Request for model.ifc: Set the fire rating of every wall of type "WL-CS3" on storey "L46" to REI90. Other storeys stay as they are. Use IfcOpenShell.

First a look at what the model holds.

```python
import ifcopenshell
import ifcopenshell.util.element

model = ifcopenshell.open("model.ifc")
print(model.schema)
storey = next(s for s in model.by_type("IfcBuildingStorey") if s.Name == "L46")
walls = [e for e in ifcopenshell.util.element.get_decomposition(storey) if e.is_a("IfcWall")]
seen = {}
for e in walls:
    element_type = ifcopenshell.util.element.get_type(e)
    key = (element_type.Name if element_type != e and element_type else None, ifcopenshell.util.element.get_pset(e, "Pset_WallCommon", "FireRating"))
    seen[key] = seen.get(key, 0) + 1
for (name, value), count in sorted(seen.items(), key=str):
    print(count, "x", name, "|", value)
```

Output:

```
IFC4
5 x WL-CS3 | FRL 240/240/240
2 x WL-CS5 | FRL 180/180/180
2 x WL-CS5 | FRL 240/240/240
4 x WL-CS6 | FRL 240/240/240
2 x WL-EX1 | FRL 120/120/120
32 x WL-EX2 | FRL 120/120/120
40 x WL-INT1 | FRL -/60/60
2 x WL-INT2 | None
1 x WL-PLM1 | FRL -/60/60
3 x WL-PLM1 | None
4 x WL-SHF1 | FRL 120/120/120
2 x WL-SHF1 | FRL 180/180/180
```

```python
import ifcopenshell
import ifcopenshell.api.pset
import ifcopenshell.util.element

model = ifcopenshell.open("model.ifc")

storey = next(s for s in model.by_type("IfcBuildingStorey") if s.Name == "L46")
walls = [e for e in ifcopenshell.util.element.get_decomposition(storey) if e.is_a("IfcWall")]

count = 0
for e in walls:
    element_type = ifcopenshell.util.element.get_type(e)
    if element_type in (None, e) or element_type.Name != "WL-CS3":
        continue
    found = ifcopenshell.util.element.get_pset(e, "Pset_WallCommon", should_inherit=False)
    if found:
        pset = model.by_id(found["id"])
        if len(ifcopenshell.util.element.get_elements_by_pset(pset)) > 1:
            pset = ifcopenshell.api.pset.unshare_pset(model, products=[e], pset=pset)[0]
    else:
        pset = ifcopenshell.api.pset.add_pset(model, product=e, name="Pset_WallCommon")
    ifcopenshell.api.pset.edit_pset(model, pset=pset, properties={"FireRating": "REI90"})
    count += 1

print(count, "walls updated")

model.write("model_updated.ifc")
```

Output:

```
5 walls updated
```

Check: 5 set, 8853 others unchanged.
